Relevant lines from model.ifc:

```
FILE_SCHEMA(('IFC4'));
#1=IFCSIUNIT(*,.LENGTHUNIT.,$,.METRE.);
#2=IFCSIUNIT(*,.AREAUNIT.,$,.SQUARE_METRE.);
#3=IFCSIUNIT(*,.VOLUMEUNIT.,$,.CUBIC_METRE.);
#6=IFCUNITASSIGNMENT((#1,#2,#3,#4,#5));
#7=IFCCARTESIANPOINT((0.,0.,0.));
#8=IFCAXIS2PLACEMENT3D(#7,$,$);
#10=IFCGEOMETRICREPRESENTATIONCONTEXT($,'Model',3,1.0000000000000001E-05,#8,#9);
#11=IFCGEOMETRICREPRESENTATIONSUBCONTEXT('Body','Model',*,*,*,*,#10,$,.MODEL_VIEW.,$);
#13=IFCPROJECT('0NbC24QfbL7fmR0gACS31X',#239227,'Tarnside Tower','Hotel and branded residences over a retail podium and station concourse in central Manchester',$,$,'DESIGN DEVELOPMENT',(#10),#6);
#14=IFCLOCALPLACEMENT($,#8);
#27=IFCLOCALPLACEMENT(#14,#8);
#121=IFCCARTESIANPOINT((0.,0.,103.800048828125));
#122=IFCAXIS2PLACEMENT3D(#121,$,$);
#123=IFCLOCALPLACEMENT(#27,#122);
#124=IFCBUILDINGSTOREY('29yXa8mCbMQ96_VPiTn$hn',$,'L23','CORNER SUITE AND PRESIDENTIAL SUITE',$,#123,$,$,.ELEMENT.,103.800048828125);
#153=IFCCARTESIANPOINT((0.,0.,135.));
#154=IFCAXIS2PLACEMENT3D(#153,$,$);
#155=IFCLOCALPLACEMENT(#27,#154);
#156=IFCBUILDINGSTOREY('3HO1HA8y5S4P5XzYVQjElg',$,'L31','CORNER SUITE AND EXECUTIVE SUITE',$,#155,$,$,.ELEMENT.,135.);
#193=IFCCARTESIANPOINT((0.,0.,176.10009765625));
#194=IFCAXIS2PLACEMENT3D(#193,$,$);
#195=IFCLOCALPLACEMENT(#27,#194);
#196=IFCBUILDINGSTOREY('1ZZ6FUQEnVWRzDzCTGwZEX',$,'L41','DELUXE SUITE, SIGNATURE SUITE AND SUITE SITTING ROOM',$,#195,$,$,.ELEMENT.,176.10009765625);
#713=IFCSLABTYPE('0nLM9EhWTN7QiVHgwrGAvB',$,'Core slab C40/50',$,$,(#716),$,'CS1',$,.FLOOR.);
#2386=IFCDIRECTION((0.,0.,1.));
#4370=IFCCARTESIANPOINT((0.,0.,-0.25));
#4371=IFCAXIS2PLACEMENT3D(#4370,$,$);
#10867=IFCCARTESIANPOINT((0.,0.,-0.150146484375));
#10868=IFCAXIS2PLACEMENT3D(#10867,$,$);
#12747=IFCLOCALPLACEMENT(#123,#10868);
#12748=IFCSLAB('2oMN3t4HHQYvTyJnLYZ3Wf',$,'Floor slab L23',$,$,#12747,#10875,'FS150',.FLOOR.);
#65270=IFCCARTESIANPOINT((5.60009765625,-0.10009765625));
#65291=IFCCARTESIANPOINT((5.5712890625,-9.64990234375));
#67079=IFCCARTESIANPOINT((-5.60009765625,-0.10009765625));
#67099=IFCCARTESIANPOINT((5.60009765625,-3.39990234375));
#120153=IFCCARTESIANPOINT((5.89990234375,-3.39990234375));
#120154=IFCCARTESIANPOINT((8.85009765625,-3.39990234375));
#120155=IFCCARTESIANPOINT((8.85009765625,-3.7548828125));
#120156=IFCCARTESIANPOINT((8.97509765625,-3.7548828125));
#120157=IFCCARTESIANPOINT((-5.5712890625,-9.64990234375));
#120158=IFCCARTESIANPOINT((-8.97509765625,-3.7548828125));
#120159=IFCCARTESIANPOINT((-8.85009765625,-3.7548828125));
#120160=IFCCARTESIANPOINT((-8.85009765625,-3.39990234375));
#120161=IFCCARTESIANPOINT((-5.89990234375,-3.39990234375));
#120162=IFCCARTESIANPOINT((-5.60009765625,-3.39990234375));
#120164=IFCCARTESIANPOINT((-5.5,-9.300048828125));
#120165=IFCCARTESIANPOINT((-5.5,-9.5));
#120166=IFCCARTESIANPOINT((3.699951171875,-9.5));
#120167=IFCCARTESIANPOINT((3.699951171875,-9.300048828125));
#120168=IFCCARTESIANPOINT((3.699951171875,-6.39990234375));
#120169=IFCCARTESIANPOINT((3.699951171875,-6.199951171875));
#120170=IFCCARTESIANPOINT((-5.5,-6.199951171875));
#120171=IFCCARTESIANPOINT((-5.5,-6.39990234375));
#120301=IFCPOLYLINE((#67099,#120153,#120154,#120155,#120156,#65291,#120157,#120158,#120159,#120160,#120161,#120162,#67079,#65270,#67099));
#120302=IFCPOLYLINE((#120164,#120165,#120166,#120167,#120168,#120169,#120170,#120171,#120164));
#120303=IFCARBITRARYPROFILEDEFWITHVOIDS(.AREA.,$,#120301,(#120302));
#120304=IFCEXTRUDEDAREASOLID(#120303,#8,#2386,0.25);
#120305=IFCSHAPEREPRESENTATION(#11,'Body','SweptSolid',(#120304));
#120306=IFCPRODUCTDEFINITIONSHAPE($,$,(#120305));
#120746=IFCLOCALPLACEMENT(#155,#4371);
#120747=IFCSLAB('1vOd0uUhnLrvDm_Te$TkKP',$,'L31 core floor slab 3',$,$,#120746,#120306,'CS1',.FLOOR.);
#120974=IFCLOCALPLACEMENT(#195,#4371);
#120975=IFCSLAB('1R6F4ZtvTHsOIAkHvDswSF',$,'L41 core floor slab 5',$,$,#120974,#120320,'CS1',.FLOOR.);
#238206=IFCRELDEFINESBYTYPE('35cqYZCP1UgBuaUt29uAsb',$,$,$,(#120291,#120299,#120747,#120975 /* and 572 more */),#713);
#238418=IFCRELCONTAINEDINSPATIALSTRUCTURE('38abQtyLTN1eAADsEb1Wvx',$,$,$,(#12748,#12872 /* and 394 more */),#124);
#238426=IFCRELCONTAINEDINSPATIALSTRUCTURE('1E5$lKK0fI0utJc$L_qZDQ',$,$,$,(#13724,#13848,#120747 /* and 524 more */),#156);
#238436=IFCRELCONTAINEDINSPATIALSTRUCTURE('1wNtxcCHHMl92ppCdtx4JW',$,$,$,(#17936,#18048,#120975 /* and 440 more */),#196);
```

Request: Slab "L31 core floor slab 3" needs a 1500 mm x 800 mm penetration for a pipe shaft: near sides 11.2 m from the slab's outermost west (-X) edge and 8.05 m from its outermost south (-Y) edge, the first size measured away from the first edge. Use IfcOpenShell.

```python
import numpy as np
import ifcopenshell
import ifcopenshell.api.feature
import ifcopenshell.api.geometry
import ifcopenshell.api.root
import ifcopenshell.geom
import ifcopenshell.util.placement
import ifcopenshell.util.representation
import ifcopenshell.util.shape
import ifcopenshell.util.unit

model = ifcopenshell.open("model.ifc")
unit_scale = ifcopenshell.util.unit.calculate_unit_scale(model)
settings = ifcopenshell.geom.settings()


def volume(element):
    """Net volume in cubic metres, openings subtracted."""
    shape = ifcopenshell.geom.create_shape(settings, element)
    return ifcopenshell.util.shape.get_volume(shape.geometry)


slab = model.by_guid("1vOd0uUhnLrvDm_Te$TkKP")
before = volume(slab)

# Extent in the slab's own axes, in metres. The edges named are its -X and -Y sides.
slab_shape = ifcopenshell.geom.create_shape(settings, slab)
vertices = ifcopenshell.util.shape.get_vertices(slab_shape.geometry)
x_min, y_min, bottom = vertices.min(axis=0)
top = vertices[:, 2].max()

opening = ifcopenshell.api.root.create_entity(model, ifc_class="IfcOpeningElement", name="Pipe shaft opening", predefined_type="OPENING")
context = ifcopenshell.util.representation.get_context(model, "Model", "Body", "MODEL_VIEW")
width, depth = 1.5, 0.8
outline = [(0.0, 0.0), (width, 0.0), (width, depth), (0.0, depth), (0.0, 0.0)]
# Overshoot both faces by 50 mm so the cut is clean.
shape = ifcopenshell.api.geometry.add_slab_representation(
    model, context=context, depth=top - bottom + 0.1, polyline=outline
)
ifcopenshell.api.geometry.assign_representation(model, product=opening, representation=shape)

matrix = ifcopenshell.util.placement.get_local_placement(slab.ObjectPlacement)
matrix[:, 3] = matrix @ np.append(np.array([x_min + 11.2, y_min + 8.05, bottom - 0.05]) / unit_scale, 1.0)
ifcopenshell.api.geometry.edit_object_placement(model, product=opening, matrix=matrix, is_si=False)
ifcopenshell.api.feature.add_feature(model, feature=opening, element=slab)

after = volume(slab)

print(f"slab volume {before:.3f} -> {after:.3f} m3")

model.write("model_edited.ifc")
```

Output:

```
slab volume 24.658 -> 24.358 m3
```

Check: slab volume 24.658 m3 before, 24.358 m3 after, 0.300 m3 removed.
